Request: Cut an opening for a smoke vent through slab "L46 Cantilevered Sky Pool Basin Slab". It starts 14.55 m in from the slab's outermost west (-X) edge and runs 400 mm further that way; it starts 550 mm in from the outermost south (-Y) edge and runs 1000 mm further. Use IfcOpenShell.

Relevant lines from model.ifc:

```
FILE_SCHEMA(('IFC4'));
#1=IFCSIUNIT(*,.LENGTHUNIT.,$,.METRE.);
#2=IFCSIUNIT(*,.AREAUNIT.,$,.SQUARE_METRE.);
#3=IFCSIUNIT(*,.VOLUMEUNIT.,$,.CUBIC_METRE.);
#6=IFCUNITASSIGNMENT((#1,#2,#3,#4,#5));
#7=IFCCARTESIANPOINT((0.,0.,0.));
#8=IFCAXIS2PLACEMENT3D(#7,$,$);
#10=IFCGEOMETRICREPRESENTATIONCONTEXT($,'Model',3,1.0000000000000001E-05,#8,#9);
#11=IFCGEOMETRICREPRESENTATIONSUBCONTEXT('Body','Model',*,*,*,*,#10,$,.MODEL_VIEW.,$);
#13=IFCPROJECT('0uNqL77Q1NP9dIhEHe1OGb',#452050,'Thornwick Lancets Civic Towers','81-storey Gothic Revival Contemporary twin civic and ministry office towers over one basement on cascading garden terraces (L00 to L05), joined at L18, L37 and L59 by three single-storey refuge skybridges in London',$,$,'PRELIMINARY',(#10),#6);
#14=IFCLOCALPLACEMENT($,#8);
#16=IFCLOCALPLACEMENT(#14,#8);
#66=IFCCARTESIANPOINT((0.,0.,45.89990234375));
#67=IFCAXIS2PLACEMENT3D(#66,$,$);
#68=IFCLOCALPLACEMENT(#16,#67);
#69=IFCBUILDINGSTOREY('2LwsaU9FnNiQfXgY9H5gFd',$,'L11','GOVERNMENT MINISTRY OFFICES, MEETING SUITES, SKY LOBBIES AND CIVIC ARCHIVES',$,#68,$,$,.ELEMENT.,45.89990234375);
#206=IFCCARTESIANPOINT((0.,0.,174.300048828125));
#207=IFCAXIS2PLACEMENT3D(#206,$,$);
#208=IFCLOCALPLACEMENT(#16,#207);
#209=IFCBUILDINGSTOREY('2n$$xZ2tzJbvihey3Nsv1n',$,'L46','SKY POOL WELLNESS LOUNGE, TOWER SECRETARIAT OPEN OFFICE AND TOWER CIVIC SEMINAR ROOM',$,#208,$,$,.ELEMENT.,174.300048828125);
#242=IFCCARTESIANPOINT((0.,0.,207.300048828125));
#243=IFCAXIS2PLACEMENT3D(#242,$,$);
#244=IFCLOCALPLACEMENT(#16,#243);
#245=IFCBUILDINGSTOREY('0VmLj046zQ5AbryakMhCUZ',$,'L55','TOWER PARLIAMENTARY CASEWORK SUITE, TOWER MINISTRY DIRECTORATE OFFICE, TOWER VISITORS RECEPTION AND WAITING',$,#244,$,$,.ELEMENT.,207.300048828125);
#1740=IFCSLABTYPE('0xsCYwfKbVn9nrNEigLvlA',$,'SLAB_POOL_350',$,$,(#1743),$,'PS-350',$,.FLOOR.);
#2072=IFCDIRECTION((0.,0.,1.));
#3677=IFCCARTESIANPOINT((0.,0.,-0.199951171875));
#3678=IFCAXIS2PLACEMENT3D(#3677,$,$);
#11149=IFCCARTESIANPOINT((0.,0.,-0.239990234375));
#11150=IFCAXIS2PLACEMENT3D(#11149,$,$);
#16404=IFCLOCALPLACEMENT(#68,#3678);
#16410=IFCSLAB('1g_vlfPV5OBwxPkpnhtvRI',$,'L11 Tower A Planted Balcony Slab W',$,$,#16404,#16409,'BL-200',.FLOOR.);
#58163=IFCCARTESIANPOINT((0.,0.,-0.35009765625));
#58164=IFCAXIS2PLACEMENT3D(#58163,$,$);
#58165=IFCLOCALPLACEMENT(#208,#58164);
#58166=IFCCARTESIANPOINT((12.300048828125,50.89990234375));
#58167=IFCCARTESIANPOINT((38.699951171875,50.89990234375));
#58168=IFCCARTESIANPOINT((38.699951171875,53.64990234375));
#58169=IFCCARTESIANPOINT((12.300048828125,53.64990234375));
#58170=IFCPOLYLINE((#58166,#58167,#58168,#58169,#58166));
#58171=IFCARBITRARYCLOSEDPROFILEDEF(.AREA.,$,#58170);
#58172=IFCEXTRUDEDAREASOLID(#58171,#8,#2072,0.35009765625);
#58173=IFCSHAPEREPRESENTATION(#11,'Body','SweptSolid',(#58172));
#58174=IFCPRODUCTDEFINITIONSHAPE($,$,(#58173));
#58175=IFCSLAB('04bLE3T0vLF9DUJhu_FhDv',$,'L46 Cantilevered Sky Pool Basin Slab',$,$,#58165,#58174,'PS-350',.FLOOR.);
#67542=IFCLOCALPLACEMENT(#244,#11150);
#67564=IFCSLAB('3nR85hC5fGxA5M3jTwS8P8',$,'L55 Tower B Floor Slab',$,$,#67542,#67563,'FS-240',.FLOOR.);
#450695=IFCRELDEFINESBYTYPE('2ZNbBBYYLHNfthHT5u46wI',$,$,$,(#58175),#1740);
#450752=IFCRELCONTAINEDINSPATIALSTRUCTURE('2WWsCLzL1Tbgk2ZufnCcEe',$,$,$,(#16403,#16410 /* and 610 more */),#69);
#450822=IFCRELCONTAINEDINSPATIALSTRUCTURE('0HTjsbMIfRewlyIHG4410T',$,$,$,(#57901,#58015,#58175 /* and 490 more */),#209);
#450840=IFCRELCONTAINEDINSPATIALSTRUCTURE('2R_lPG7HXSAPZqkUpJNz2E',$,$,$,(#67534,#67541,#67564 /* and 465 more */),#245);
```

```python
import numpy as np
import ifcopenshell
import ifcopenshell.api.feature
import ifcopenshell.api.geometry
import ifcopenshell.api.root
import ifcopenshell.geom
import ifcopenshell.util.placement
import ifcopenshell.util.representation
import ifcopenshell.util.shape
import ifcopenshell.util.unit

model = ifcopenshell.open("model.ifc")
unit_scale = ifcopenshell.util.unit.calculate_unit_scale(model)
settings = ifcopenshell.geom.settings()


def volume(element):
    """Net volume in cubic metres, openings subtracted."""
    shape = ifcopenshell.geom.create_shape(settings, element)
    return ifcopenshell.util.shape.get_volume(shape.geometry)


slab = model.by_guid("04bLE3T0vLF9DUJhu_FhDv")
before = volume(slab)

# Extent in the slab's own axes, in metres. The edges named are its -X and -Y sides.
slab_shape = ifcopenshell.geom.create_shape(settings, slab)
vertices = ifcopenshell.util.shape.get_vertices(slab_shape.geometry)
x_min, y_min, bottom = vertices.min(axis=0)
top = vertices[:, 2].max()

opening = ifcopenshell.api.root.create_entity(model, ifc_class="IfcOpeningElement", name="Smoke vent opening", predefined_type="OPENING")
context = ifcopenshell.util.representation.get_context(model, "Model", "Body", "MODEL_VIEW")
width, depth = 0.4, 1
outline = [(0.0, 0.0), (width, 0.0), (width, depth), (0.0, depth), (0.0, 0.0)]
# Overshoot both faces by 50 mm so the cut is clean.
shape = ifcopenshell.api.geometry.add_slab_representation(
    model, context=context, depth=top - bottom + 0.1, polyline=outline
)
ifcopenshell.api.geometry.assign_representation(model, product=opening, representation=shape)

matrix = ifcopenshell.util.placement.get_local_placement(slab.ObjectPlacement)
matrix[:, 3] = matrix @ np.append(np.array([x_min + 14.55, y_min + 0.55, bottom - 0.05]) / unit_scale, 1.0)
ifcopenshell.api.geometry.edit_object_placement(model, product=opening, matrix=matrix, is_si=False)
ifcopenshell.api.feature.add_feature(model, feature=opening, element=slab)

after = volume(slab)

print(f"slab volume {before:.3f} -> {after:.3f} m3")

model.write("model_edited.ifc")
```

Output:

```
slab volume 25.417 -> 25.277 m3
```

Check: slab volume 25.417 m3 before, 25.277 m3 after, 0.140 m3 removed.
